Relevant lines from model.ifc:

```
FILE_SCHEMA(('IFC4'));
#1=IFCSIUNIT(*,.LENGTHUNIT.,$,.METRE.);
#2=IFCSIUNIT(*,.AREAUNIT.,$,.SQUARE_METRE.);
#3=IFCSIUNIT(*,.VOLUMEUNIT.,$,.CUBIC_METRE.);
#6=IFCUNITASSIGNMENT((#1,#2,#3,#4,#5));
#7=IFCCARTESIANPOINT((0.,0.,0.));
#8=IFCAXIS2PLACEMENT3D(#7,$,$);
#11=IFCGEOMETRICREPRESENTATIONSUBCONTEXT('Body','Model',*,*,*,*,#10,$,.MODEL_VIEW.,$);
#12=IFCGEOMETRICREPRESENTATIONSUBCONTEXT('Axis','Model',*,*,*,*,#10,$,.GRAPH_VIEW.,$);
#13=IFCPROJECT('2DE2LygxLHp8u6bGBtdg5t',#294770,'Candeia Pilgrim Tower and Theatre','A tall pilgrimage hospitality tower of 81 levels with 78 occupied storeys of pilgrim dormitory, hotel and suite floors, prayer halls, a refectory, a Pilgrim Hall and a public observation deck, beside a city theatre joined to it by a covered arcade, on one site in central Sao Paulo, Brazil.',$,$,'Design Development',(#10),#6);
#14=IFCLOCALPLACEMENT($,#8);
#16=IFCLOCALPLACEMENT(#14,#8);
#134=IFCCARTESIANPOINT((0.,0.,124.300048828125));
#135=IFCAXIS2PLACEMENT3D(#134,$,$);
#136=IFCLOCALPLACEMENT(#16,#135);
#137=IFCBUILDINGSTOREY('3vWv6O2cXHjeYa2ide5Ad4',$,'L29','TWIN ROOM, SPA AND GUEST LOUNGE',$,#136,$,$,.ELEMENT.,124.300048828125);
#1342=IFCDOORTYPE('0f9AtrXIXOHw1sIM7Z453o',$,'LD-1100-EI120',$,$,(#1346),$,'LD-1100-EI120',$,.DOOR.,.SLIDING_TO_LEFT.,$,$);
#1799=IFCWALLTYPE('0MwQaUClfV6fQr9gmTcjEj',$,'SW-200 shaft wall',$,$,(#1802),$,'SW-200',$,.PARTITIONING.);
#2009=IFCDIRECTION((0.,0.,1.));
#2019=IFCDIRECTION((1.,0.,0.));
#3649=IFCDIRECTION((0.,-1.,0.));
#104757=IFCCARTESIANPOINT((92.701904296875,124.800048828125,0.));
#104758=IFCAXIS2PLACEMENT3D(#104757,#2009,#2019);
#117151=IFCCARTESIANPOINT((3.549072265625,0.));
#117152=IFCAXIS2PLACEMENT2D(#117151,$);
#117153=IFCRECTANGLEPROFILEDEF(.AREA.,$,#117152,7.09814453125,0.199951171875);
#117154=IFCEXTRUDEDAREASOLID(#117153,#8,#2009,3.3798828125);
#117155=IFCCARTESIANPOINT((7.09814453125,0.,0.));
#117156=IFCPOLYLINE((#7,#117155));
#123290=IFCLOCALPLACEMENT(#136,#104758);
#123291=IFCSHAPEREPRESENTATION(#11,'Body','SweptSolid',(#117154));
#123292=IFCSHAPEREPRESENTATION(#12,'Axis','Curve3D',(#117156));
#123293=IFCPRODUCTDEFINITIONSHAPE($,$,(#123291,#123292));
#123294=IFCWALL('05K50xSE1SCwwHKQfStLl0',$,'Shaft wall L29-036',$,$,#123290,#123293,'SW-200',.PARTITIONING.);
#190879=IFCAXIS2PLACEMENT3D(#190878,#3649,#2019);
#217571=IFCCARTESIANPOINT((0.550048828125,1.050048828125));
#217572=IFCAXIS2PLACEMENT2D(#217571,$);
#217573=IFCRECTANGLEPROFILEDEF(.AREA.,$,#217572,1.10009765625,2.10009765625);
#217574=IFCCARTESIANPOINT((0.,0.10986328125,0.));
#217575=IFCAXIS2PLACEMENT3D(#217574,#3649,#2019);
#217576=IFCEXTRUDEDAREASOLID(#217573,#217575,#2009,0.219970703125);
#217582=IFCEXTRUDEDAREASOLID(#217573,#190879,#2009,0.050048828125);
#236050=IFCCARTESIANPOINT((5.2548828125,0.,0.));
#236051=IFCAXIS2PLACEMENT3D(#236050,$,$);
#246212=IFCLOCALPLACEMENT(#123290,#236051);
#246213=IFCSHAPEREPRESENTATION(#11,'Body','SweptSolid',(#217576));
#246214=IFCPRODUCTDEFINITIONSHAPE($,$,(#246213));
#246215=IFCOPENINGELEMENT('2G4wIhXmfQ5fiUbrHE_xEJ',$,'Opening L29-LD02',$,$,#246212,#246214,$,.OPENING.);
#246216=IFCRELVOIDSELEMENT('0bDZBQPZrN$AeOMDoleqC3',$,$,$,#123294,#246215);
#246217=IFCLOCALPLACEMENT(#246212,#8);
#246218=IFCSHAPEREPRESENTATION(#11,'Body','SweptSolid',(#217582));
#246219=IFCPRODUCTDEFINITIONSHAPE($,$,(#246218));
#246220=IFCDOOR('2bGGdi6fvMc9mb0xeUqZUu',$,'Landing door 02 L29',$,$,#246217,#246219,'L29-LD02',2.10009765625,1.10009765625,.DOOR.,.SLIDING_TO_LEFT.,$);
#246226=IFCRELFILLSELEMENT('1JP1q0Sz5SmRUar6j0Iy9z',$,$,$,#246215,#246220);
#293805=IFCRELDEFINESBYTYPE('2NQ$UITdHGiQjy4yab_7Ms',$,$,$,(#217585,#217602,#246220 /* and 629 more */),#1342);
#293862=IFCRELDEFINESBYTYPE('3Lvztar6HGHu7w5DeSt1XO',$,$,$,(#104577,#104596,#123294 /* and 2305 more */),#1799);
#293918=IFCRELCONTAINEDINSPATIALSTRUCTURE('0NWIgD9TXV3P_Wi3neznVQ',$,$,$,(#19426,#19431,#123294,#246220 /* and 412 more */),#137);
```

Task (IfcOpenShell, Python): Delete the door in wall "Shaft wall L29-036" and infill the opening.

```python
import ifcopenshell
import ifcopenshell.api.feature
import ifcopenshell.api.root
import ifcopenshell.geom
import ifcopenshell.util.shape

model = ifcopenshell.open("model.ifc")
settings = ifcopenshell.geom.settings()


def volume(element):
    """Net volume in cubic metres, openings subtracted."""
    shape = ifcopenshell.geom.create_shape(settings, element)
    return ifcopenshell.util.shape.get_volume(shape.geometry)


door = model.by_id(246220)
opening = door.FillsVoids[0].RelatingOpeningElement
wall = opening.VoidsElements[0].RelatingBuildingElement
before = volume(wall)

ifcopenshell.api.root.remove_product(model, product=door)
ifcopenshell.api.feature.remove_feature(model, feature=opening)

after = volume(wall)

print(f"wall volume {before:.3f} -> {after:.3f} m3")

model.write("model_v2.ifc")
```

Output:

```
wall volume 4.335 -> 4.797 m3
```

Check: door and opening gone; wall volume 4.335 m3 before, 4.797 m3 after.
